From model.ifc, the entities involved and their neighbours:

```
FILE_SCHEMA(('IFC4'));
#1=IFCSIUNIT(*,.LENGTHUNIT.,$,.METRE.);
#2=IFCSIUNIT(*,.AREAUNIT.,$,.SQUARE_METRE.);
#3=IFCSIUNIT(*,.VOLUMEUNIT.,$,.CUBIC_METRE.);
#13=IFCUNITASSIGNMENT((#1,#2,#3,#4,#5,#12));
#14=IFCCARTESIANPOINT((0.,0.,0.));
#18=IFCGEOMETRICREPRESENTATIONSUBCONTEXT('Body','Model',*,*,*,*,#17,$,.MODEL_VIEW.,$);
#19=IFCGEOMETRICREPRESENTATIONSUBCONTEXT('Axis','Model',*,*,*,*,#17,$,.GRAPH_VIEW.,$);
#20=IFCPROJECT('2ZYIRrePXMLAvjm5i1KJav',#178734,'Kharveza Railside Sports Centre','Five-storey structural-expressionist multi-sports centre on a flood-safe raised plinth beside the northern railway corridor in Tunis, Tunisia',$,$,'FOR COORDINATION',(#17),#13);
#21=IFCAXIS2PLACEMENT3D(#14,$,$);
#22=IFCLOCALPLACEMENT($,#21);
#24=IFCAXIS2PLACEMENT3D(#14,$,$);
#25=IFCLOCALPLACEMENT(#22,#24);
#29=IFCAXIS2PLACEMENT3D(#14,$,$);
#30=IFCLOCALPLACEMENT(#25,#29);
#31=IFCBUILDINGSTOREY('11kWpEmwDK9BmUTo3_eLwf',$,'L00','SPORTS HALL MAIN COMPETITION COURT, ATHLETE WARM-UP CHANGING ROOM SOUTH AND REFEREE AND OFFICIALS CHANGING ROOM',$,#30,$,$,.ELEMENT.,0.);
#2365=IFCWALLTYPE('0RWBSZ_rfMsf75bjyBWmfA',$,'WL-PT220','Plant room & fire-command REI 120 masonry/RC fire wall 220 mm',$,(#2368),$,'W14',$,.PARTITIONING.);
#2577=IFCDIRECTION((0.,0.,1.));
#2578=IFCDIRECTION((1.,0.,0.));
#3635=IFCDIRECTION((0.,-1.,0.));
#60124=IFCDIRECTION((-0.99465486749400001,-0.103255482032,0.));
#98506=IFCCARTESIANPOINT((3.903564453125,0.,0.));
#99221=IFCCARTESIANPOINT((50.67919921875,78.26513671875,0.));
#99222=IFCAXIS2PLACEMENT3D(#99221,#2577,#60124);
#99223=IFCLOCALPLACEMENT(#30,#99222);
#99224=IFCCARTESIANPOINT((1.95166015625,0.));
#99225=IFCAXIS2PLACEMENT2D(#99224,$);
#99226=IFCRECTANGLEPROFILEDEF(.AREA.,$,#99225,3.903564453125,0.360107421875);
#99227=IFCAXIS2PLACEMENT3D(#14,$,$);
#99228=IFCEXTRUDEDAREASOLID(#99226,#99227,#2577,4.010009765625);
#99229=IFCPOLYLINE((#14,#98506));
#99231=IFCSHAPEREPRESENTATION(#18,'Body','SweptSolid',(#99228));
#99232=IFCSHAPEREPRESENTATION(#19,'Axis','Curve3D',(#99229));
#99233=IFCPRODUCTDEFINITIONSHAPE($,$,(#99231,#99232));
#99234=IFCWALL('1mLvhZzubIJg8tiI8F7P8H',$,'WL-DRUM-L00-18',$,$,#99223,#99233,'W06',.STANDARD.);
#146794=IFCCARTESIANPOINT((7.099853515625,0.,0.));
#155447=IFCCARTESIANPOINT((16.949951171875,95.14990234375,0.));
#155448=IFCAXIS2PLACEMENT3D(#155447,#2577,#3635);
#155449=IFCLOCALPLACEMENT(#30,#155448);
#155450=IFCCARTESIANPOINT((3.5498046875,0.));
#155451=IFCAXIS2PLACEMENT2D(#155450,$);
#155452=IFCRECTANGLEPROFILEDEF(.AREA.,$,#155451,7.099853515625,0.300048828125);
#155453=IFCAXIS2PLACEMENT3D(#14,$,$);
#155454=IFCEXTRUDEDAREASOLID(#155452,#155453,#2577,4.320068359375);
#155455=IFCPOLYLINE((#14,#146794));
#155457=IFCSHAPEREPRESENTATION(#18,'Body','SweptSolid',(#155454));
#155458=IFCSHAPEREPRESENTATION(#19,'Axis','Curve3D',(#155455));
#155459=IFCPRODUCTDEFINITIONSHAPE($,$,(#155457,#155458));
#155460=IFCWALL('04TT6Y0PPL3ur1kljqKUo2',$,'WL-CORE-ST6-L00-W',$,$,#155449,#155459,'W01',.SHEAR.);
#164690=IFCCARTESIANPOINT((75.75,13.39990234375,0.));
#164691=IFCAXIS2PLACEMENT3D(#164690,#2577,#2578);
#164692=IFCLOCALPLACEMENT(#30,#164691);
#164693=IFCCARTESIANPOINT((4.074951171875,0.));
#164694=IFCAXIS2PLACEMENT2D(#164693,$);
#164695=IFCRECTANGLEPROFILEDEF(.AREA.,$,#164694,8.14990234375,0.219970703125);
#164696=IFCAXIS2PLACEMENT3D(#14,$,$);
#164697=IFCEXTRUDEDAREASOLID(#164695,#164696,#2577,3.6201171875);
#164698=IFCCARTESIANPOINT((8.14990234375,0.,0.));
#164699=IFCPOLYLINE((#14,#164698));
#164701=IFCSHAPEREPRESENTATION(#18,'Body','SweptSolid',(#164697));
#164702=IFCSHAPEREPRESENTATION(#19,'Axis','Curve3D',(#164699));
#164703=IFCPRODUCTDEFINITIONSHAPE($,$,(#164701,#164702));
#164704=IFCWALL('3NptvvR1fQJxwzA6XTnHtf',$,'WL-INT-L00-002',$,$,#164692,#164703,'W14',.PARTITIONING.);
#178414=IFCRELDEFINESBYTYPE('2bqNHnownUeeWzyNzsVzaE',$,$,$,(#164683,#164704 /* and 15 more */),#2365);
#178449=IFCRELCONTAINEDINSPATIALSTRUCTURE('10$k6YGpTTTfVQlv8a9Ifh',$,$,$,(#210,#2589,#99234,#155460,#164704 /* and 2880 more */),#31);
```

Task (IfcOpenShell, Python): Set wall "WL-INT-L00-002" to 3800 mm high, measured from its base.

```python
import ifcopenshell
import ifcopenshell.geom
import ifcopenshell.util.representation
import ifcopenshell.util.shape
import ifcopenshell.util.unit

model = ifcopenshell.open("model.ifc")
unit_scale = ifcopenshell.util.unit.calculate_unit_scale(model)
settings = ifcopenshell.geom.settings()


def volume(element):
    """Net volume in cubic metres, openings subtracted."""
    shape = ifcopenshell.geom.create_shape(settings, element)
    return ifcopenshell.util.shape.get_volume(shape.geometry)


wall = model.by_id(164704)
before = volume(wall)

body = ifcopenshell.util.representation.get_representation(wall, "Model", "Body")
solid = body.Items[0]
old_height = solid.Depth
solid.Depth = 3.8 / unit_scale
after = volume(wall)

print(f"height {old_height:g} -> {solid.Depth:g}, volume {before:.3f} -> {after:.3f} m3")

model.write("model_updated.ifc")
```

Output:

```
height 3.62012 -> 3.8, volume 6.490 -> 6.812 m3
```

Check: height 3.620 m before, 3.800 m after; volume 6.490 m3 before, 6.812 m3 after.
